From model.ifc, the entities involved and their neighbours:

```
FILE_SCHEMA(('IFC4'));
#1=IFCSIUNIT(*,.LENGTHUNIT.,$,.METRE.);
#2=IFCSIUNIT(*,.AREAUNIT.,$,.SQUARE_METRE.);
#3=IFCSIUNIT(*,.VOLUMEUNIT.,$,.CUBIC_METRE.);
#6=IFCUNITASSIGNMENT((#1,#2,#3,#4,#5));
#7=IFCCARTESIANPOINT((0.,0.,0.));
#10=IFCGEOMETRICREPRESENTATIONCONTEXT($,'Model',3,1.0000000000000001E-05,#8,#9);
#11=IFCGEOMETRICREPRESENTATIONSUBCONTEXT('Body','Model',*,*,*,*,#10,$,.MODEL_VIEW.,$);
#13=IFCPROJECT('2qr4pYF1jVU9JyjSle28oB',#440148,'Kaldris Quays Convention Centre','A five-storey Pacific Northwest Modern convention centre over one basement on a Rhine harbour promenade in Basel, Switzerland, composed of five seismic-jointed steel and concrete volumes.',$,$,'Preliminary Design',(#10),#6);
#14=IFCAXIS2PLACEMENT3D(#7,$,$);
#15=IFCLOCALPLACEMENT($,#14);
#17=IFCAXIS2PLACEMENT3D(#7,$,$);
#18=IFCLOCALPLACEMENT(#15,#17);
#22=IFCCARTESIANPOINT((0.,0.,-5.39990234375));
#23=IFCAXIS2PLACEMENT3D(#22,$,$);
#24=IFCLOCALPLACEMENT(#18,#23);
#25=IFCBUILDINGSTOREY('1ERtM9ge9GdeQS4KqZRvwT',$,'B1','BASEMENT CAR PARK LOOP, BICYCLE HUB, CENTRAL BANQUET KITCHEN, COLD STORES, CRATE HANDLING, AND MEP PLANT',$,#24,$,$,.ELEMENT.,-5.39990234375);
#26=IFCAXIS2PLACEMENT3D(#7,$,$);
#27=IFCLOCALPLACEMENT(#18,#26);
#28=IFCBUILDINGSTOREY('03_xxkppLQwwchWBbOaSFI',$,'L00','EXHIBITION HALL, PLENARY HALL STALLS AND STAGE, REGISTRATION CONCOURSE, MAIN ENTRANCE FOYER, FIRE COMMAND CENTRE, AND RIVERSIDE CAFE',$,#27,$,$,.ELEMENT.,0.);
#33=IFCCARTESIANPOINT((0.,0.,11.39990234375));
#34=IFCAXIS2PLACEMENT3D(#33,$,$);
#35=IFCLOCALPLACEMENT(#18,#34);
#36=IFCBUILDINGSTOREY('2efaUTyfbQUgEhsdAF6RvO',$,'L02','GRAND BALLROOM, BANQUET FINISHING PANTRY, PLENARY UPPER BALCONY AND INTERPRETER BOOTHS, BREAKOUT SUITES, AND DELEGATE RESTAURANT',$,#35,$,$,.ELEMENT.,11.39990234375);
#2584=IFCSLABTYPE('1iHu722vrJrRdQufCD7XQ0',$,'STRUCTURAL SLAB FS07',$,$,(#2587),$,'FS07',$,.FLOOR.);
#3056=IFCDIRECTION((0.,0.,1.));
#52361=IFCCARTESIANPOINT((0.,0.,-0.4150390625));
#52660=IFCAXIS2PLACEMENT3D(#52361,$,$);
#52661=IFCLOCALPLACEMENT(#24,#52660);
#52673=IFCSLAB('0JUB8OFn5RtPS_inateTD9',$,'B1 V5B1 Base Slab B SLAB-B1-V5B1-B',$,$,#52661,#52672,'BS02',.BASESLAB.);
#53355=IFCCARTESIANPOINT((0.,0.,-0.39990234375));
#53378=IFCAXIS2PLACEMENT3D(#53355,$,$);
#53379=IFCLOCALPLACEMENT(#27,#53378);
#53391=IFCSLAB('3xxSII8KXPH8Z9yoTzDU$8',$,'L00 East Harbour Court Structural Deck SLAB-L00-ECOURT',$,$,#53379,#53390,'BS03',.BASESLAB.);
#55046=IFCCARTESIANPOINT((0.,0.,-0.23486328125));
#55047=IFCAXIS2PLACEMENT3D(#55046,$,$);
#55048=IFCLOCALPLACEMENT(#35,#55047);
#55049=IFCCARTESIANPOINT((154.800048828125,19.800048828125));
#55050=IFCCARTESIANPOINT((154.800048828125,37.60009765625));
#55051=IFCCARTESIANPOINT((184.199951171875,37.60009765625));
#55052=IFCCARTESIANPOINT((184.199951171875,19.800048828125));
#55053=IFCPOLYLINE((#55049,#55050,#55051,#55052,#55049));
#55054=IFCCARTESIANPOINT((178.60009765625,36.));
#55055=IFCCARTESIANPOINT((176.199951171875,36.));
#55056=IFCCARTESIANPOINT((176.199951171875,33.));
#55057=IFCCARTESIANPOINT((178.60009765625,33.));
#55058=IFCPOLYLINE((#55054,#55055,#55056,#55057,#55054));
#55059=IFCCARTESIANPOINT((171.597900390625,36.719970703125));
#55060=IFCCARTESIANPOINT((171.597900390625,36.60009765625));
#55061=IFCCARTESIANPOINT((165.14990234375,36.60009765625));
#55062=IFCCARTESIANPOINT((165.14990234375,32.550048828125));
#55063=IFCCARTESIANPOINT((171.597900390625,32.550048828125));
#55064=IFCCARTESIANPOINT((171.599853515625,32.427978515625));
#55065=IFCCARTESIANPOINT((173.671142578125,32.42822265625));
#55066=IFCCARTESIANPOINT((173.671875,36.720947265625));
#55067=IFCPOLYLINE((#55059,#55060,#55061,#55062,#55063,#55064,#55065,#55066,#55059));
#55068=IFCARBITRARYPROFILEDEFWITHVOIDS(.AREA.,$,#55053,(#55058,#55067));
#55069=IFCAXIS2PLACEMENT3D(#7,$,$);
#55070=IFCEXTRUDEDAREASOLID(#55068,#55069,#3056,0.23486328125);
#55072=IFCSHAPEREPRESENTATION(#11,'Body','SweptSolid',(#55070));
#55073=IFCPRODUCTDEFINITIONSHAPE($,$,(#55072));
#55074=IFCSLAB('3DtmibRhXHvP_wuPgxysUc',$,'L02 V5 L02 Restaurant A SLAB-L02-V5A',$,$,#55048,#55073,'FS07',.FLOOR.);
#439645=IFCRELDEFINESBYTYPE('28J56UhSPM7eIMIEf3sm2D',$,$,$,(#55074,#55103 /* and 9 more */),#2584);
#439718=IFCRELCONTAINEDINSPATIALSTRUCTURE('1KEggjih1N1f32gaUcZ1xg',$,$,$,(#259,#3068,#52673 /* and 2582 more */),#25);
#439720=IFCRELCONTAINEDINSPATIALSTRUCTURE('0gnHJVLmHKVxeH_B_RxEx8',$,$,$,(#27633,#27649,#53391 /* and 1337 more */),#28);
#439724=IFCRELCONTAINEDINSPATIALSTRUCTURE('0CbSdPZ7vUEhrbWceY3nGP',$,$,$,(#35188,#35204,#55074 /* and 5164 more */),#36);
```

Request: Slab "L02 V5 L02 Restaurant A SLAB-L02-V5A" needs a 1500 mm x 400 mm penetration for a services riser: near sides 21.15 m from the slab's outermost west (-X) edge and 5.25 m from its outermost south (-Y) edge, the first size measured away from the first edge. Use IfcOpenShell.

```python
import numpy as np
import ifcopenshell
import ifcopenshell.api.feature
import ifcopenshell.api.geometry
import ifcopenshell.api.root
import ifcopenshell.geom
import ifcopenshell.util.placement
import ifcopenshell.util.representation
import ifcopenshell.util.shape
import ifcopenshell.util.unit

model = ifcopenshell.open("model.ifc")
unit_scale = ifcopenshell.util.unit.calculate_unit_scale(model)
settings = ifcopenshell.geom.settings()


def volume(element):
    """Net volume in cubic metres, openings subtracted."""
    shape = ifcopenshell.geom.create_shape(settings, element)
    return ifcopenshell.util.shape.get_volume(shape.geometry)


slab = model.by_id(55074)
before = volume(slab)

# Extent in the slab's own axes, in metres. The edges named are its -X and -Y sides.
slab_shape = ifcopenshell.geom.create_shape(settings, slab)
vertices = ifcopenshell.util.shape.get_vertices(slab_shape.geometry)
x_min, y_min, bottom = vertices.min(axis=0)
top = vertices[:, 2].max()

opening = ifcopenshell.api.root.create_entity(model, ifc_class="IfcOpeningElement", name="Services riser opening", predefined_type="OPENING")
context = ifcopenshell.util.representation.get_context(model, "Model", "Body", "MODEL_VIEW")
width, depth = 1.5, 0.4
outline = [(0.0, 0.0), (width, 0.0), (width, depth), (0.0, depth), (0.0, 0.0)]
# Overshoot both faces by 50 mm so the cut is clean.
shape = ifcopenshell.api.geometry.add_slab_representation(
    model, context=context, depth=top - bottom + 0.1, polyline=outline
)
ifcopenshell.api.geometry.assign_representation(model, product=opening, representation=shape)

matrix = ifcopenshell.util.placement.get_local_placement(slab.ObjectPlacement)
matrix[:, 3] = matrix @ np.append(np.array([x_min + 21.15, y_min + 5.25, bottom - 0.05]) / unit_scale, 1.0)
ifcopenshell.api.geometry.edit_object_placement(model, product=opening, matrix=matrix, is_si=False)
ifcopenshell.api.feature.add_feature(model, feature=opening, element=slab)

after = volume(slab)

print(f"slab volume {before:.3f} -> {after:.3f} m3")

model.write("model_rev.ifc")
```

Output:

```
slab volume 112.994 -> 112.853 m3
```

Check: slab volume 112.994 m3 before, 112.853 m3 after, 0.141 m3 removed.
